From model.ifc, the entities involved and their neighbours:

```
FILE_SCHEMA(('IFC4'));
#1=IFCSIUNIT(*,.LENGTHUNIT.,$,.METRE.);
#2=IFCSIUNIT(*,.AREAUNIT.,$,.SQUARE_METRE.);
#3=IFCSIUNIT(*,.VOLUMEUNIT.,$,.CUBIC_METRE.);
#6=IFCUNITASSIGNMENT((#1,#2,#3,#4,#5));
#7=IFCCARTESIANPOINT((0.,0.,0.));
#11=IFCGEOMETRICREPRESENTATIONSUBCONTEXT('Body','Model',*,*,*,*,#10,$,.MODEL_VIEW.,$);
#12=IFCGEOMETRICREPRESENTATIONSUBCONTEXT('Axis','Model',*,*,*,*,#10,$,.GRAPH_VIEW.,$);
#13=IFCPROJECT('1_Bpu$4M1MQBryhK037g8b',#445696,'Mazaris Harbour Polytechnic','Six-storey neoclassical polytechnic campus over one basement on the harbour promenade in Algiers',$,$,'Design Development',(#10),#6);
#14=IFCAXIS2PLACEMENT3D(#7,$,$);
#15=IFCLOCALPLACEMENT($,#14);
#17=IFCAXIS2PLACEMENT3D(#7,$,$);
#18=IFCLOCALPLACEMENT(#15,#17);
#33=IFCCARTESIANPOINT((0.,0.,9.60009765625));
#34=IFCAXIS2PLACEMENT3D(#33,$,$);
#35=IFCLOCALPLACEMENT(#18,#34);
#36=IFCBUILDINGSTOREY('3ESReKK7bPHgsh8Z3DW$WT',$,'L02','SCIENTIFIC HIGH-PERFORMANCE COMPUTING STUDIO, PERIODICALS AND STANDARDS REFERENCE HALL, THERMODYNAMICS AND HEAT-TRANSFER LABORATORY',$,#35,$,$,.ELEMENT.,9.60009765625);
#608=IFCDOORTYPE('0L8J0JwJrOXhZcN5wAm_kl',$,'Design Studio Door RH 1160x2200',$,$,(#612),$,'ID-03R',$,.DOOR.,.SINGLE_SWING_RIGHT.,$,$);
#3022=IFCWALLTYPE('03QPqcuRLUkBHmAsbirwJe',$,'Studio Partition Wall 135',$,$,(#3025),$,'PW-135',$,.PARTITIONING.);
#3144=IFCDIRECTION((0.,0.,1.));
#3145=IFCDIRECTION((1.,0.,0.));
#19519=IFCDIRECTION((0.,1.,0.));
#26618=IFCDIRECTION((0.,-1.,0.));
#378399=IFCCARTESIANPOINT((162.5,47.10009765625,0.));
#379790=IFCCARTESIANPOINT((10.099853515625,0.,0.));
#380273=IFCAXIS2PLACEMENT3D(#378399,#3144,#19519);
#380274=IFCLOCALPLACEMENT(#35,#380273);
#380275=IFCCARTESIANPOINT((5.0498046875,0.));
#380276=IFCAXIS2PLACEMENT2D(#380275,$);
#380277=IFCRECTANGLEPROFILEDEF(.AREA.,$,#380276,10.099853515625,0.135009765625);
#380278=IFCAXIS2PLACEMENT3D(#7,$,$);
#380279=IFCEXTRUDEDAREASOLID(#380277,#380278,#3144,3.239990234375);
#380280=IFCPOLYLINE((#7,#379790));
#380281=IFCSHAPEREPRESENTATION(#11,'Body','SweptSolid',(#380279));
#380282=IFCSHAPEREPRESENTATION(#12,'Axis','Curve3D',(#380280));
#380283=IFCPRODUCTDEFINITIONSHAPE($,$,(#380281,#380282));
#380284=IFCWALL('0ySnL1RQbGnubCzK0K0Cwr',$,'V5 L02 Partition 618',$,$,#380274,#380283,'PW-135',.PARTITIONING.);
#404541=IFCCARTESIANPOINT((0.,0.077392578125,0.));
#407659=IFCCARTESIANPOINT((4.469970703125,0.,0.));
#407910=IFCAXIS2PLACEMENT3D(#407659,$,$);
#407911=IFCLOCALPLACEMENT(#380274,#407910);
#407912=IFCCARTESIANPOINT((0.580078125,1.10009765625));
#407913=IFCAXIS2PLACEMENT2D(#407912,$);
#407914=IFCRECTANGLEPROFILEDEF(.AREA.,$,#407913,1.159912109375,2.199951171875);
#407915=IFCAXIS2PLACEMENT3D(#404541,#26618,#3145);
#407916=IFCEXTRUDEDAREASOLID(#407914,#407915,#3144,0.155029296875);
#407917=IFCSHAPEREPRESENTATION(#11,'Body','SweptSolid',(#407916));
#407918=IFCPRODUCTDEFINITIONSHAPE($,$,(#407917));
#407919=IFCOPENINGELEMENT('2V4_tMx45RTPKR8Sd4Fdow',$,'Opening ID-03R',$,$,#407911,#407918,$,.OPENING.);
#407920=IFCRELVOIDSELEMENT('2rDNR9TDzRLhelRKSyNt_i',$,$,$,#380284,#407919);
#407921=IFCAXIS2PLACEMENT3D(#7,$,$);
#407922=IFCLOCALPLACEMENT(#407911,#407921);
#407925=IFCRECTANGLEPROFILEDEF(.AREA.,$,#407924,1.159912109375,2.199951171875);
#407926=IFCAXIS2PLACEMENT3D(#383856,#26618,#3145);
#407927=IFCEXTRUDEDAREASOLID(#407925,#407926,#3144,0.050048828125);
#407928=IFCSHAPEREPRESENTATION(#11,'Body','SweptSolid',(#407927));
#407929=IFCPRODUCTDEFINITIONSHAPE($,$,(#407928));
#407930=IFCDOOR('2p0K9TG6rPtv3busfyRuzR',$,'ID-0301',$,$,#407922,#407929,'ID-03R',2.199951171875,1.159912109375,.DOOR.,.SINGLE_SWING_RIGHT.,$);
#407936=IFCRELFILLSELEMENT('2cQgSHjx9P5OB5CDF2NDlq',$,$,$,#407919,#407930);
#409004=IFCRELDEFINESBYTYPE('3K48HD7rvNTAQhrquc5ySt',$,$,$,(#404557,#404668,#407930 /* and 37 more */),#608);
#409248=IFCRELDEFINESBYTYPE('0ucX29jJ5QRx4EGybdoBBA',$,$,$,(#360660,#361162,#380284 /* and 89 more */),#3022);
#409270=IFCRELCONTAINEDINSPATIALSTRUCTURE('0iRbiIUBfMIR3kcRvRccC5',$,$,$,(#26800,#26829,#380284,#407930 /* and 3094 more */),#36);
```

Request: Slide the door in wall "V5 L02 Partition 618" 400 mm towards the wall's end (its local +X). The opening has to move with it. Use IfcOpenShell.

```python
import ifcopenshell
import ifcopenshell.api.geometry
import ifcopenshell.util.placement

model = ifcopenshell.open("model.ifc")

door = model.by_guid("2p0K9TG6rPtv3busfyRuzR")
opening = door.FillsVoids[0].RelatingOpeningElement
wall = opening.VoidsElements[0].RelatingBuildingElement

wall_matrix = ifcopenshell.util.placement.get_local_placement(wall.ObjectPlacement)
shift = wall_matrix[:3, 0] * 0.4
before = ifcopenshell.util.placement.get_local_placement(door.ObjectPlacement)[:3, 3].copy()

# The door is placed relative to its opening, so it follows when the opening moves.
matrix = ifcopenshell.util.placement.get_local_placement(opening.ObjectPlacement)
matrix[:3, 3] += shift
ifcopenshell.api.geometry.edit_object_placement(
    model, product=opening, matrix=matrix, is_si=False, should_transform_children=True
)

after = ifcopenshell.util.placement.get_local_placement(door.ObjectPlacement)[:3, 3]
print("door moved by", (after - before).round(3) + 0.0)

model.write("model_edited.ifc")
```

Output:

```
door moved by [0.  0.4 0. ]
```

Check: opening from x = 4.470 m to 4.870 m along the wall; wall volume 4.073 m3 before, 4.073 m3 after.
